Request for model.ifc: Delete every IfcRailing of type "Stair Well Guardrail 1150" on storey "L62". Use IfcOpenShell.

First a look at what the model holds.

```python
import ifcopenshell
import ifcopenshell.util.element

model = ifcopenshell.open("model.ifc")
print(model.schema)
storey = next(s for s in model.by_type("IfcBuildingStorey") if s.Name == "L62")
railings = [e for e in ifcopenshell.util.element.get_decomposition(storey) if e.is_a("IfcRailing")]
seen = {}
for e in railings:
    element_type = ifcopenshell.util.element.get_type(e)
    name = element_type.Name if element_type not in (None, e) else None
    seen[name] = seen.get(name, 0) + 1
for name, count in sorted(seen.items(), key=str):
    print(count, "x", name)
```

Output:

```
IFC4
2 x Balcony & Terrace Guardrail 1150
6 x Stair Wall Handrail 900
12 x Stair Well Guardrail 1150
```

```python
import ifcopenshell
import ifcopenshell.api.root
import ifcopenshell.util.element

model = ifcopenshell.open("model.ifc")

storey = next(s for s in model.by_type("IfcBuildingStorey") if s.Name == "L62")
railings = [e for e in ifcopenshell.util.element.get_decomposition(storey) if e.is_a("IfcRailing")]
targets = [e for e in railings if (t := ifcopenshell.util.element.get_type(e)) not in (None, e) and t.Name == "Stair Well Guardrail 1150"]

for e in targets:
    ifcopenshell.api.root.remove_product(model, product=e)
print(len(targets), "removed")

model.write("model_rev.ifc")
```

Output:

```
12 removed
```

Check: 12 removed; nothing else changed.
